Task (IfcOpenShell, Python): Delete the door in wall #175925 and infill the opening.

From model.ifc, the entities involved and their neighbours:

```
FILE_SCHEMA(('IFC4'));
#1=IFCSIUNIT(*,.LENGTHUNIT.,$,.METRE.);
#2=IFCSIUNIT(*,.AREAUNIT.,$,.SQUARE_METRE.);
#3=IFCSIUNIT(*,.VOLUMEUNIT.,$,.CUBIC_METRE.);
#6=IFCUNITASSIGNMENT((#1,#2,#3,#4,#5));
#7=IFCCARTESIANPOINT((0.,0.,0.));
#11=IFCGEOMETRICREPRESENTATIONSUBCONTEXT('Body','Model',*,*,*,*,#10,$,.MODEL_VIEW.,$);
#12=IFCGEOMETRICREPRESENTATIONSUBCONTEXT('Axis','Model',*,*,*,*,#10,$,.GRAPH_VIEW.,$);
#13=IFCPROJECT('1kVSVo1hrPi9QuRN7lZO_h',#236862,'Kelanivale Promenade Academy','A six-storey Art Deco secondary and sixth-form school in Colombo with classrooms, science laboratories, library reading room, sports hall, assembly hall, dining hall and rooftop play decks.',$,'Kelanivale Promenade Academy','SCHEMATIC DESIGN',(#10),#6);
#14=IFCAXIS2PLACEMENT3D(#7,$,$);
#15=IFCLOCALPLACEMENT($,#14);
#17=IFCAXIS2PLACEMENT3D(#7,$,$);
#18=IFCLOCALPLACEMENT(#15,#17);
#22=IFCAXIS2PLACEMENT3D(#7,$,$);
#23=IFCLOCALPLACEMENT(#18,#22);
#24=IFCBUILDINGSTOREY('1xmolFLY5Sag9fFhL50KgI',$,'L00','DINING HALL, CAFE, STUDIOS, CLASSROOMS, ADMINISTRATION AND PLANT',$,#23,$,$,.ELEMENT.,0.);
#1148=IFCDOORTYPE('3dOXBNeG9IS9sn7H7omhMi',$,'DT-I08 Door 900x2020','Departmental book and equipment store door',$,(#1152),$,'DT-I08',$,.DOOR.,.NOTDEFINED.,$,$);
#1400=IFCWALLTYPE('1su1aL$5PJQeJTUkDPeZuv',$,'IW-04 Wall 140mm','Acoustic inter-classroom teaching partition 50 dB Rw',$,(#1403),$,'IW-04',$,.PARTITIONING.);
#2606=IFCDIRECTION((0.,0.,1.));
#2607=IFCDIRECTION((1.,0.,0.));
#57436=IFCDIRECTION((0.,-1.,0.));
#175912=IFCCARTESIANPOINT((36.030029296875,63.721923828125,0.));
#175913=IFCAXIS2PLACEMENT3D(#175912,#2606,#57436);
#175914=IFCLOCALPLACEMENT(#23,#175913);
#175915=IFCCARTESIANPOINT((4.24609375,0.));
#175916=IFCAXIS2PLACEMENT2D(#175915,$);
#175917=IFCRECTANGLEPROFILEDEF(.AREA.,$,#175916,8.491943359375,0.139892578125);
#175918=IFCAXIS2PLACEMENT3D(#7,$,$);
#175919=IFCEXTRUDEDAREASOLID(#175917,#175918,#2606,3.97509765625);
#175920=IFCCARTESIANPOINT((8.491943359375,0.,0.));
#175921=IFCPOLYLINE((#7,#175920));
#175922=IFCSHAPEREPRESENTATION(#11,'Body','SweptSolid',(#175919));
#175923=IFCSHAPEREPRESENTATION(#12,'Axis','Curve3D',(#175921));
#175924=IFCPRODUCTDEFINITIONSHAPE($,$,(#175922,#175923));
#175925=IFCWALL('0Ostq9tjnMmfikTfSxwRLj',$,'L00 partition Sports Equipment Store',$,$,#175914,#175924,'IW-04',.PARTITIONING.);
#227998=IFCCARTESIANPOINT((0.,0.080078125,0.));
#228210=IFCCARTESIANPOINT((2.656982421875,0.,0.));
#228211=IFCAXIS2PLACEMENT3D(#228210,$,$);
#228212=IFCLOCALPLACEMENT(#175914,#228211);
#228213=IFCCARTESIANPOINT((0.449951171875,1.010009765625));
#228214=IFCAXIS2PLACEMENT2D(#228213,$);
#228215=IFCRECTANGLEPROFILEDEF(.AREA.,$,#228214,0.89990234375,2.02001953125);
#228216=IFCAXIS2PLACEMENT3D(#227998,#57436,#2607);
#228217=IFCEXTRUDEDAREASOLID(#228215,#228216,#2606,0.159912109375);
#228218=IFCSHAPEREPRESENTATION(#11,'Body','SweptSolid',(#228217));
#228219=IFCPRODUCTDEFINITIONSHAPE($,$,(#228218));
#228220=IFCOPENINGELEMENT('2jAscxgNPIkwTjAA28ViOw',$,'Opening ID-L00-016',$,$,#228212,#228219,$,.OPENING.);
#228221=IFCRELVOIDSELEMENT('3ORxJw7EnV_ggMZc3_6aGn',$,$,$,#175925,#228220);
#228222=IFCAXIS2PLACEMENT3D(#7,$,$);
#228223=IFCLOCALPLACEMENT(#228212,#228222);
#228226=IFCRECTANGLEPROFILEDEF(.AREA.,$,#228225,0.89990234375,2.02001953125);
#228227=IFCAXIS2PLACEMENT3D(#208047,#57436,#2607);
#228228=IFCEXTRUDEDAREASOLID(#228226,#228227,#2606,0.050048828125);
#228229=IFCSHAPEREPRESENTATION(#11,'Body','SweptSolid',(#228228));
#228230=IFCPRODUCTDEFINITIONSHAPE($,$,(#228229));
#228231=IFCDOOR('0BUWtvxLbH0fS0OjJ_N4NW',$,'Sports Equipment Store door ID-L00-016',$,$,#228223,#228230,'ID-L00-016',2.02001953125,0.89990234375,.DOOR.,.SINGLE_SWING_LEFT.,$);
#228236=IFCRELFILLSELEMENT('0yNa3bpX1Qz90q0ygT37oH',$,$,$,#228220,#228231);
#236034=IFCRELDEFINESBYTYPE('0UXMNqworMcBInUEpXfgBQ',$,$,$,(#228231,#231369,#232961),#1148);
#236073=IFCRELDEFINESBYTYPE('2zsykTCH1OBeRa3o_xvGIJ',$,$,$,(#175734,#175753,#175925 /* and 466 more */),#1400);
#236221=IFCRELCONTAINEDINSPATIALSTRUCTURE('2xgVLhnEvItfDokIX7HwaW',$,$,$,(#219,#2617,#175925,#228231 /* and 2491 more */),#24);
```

```python
import ifcopenshell
import ifcopenshell.api.feature
import ifcopenshell.api.root
import ifcopenshell.geom
import ifcopenshell.util.shape

model = ifcopenshell.open("model.ifc")
settings = ifcopenshell.geom.settings()


def volume(element):
    """Net volume in cubic metres, openings subtracted."""
    shape = ifcopenshell.geom.create_shape(settings, element)
    return ifcopenshell.util.shape.get_volume(shape.geometry)


door = model.by_guid("0BUWtvxLbH0fS0OjJ_N4NW")
opening = door.FillsVoids[0].RelatingOpeningElement
wall = opening.VoidsElements[0].RelatingBuildingElement
before = volume(wall)

ifcopenshell.api.root.remove_product(model, product=door)
ifcopenshell.api.feature.remove_feature(model, feature=opening)

after = volume(wall)

print(f"wall volume {before:.3f} -> {after:.3f} m3")

model.write("model_v2.ifc")
```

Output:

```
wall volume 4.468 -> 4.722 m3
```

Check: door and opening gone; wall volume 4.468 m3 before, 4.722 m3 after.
